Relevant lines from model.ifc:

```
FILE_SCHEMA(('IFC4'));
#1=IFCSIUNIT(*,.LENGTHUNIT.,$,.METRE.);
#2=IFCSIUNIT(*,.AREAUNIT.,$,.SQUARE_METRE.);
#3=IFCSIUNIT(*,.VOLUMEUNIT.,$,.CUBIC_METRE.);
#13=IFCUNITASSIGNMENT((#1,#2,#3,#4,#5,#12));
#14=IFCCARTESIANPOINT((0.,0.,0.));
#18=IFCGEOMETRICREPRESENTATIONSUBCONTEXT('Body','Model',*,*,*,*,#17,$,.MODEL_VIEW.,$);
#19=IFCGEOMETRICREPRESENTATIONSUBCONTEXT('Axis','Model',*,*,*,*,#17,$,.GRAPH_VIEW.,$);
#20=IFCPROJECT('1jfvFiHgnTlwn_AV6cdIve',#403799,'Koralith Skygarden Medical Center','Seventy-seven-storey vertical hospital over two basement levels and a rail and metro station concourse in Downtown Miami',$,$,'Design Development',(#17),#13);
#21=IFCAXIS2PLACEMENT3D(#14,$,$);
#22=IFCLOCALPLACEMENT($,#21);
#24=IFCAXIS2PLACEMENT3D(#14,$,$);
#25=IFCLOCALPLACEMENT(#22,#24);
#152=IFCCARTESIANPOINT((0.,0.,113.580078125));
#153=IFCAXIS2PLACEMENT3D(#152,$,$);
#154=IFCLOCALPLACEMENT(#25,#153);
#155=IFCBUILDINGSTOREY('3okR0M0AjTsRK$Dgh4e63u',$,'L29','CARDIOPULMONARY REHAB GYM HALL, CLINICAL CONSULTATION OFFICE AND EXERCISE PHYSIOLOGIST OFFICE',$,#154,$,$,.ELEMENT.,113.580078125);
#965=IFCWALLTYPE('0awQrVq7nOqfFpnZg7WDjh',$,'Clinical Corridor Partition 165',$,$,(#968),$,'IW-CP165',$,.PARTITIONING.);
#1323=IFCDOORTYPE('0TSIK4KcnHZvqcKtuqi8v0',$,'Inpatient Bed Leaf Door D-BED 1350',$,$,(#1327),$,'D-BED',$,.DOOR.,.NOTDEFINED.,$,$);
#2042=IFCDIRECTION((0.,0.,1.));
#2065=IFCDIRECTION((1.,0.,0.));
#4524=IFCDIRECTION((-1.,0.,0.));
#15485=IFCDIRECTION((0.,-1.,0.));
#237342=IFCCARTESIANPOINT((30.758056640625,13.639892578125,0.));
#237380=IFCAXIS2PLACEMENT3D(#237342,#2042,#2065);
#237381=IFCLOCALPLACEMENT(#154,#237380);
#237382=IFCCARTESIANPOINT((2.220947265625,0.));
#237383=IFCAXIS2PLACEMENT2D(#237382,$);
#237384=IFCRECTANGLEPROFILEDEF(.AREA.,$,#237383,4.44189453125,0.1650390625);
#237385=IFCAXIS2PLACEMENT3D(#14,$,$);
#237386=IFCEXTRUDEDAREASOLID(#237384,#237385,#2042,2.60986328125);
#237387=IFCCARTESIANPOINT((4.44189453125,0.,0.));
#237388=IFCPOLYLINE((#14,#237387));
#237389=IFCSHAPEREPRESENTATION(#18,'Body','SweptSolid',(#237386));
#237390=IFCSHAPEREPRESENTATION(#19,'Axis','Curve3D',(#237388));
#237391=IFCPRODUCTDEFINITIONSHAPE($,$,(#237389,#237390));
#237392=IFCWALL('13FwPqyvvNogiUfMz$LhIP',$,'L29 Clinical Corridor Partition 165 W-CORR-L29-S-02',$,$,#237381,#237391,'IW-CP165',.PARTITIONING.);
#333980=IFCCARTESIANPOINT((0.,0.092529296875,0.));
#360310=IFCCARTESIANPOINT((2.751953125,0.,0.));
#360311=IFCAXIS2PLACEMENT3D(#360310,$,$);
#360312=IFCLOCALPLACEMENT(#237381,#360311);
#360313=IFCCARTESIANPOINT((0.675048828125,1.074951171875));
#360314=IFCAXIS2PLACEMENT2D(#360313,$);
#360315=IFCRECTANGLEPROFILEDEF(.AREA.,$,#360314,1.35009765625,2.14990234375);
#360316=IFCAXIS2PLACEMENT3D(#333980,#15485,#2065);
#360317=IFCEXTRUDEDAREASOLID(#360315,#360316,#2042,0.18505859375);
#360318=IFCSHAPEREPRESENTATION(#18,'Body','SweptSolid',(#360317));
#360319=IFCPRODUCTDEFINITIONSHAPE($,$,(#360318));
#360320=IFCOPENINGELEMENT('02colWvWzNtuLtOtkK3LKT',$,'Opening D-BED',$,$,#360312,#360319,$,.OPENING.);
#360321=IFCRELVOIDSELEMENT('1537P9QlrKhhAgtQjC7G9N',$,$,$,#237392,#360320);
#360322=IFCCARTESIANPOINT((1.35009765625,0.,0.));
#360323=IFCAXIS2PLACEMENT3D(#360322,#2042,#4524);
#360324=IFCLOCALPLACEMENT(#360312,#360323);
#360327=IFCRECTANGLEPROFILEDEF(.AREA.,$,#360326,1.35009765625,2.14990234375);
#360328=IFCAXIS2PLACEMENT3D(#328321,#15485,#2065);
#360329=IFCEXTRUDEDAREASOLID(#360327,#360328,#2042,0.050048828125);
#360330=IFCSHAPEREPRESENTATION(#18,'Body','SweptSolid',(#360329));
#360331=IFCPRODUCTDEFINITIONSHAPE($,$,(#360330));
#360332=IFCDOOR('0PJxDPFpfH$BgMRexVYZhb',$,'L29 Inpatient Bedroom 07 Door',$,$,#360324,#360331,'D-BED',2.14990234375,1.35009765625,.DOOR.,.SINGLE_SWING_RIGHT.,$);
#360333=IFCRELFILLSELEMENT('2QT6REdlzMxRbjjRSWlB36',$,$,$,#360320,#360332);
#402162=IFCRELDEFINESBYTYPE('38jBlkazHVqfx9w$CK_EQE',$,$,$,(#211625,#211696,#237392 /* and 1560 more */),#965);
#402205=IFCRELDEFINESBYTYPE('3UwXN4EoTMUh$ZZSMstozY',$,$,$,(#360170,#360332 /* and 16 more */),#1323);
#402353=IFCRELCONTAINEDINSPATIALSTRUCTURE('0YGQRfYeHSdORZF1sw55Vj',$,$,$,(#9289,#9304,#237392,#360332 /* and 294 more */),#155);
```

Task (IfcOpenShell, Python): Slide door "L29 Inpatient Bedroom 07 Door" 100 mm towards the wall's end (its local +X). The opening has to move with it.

```python
import ifcopenshell
import ifcopenshell.api.geometry
import ifcopenshell.util.placement

model = ifcopenshell.open("model.ifc")

door = model.by_guid("0PJxDPFpfH$BgMRexVYZhb")
opening = door.FillsVoids[0].RelatingOpeningElement
wall = opening.VoidsElements[0].RelatingBuildingElement

wall_matrix = ifcopenshell.util.placement.get_local_placement(wall.ObjectPlacement)
shift = wall_matrix[:3, 0] * 0.1
before = ifcopenshell.util.placement.get_local_placement(door.ObjectPlacement)[:3, 3].copy()

# The door is placed relative to its opening, so it follows when the opening moves.
matrix = ifcopenshell.util.placement.get_local_placement(opening.ObjectPlacement)
matrix[:3, 3] += shift
ifcopenshell.api.geometry.edit_object_placement(
    model, product=opening, matrix=matrix, is_si=False, should_transform_children=True
)

after = ifcopenshell.util.placement.get_local_placement(door.ObjectPlacement)[:3, 3]
print("door moved by", (after - before).round(3) + 0.0)

model.write("model_edited.ifc")
```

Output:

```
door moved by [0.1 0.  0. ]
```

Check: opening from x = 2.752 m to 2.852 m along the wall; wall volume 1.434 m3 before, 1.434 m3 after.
